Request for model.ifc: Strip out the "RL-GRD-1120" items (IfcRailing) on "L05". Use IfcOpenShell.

First a look at what the model holds.

```python
import ifcopenshell
import ifcopenshell.util.element

model = ifcopenshell.open("model.ifc")
print(model.schema)
storey = next(s for s in model.by_type("IfcBuildingStorey") if s.Name == "L05")
railings = [e for e in ifcopenshell.util.element.get_decomposition(storey) if e.is_a("IfcRailing")]
seen = {}
for e in railings:
    element_type = ifcopenshell.util.element.get_type(e)
    name = element_type.Name if element_type not in (None, e) else None
    seen[name] = seen.get(name, 0) + 1
for name, count in sorted(seen.items(), key=str):
    print(count, "x", name)
```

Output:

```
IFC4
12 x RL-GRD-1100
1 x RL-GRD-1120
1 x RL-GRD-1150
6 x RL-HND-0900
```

```python
import ifcopenshell
import ifcopenshell.api.root
import ifcopenshell.util.element

model = ifcopenshell.open("model.ifc")

storey = next(s for s in model.by_type("IfcBuildingStorey") if s.Name == "L05")
railings = [e for e in ifcopenshell.util.element.get_decomposition(storey) if e.is_a("IfcRailing")]
targets = [e for e in railings if (t := ifcopenshell.util.element.get_type(e)) not in (None, e) and t.Name == "RL-GRD-1120"]

for e in targets:
    ifcopenshell.api.root.remove_product(model, product=e)
print(len(targets), "removed")

model.write("model_rev.ifc")
```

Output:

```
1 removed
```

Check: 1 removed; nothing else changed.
